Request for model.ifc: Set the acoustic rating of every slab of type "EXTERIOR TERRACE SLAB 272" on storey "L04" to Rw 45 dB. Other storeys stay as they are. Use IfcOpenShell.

First a look at what the model holds.

```python
import ifcopenshell
import ifcopenshell.util.element

model = ifcopenshell.open("model.ifc")
print(model.schema)
storey = next(s for s in model.by_type("IfcBuildingStorey") if s.Name == "L04")
slabs = [e for e in ifcopenshell.util.element.get_decomposition(storey) if e.is_a("IfcSlab")]
seen = {}
for e in slabs:
    element_type = ifcopenshell.util.element.get_type(e)
    key = (element_type.Name if element_type != e and element_type else None, ifcopenshell.util.element.get_pset(e, "Pset_SlabCommon", "AcousticRating"))
    seen[key] = seen.get(key, 0) + 1
for (name, value), count in sorted(seen.items(), key=str):
    print(count, "x", name, "|", value)
```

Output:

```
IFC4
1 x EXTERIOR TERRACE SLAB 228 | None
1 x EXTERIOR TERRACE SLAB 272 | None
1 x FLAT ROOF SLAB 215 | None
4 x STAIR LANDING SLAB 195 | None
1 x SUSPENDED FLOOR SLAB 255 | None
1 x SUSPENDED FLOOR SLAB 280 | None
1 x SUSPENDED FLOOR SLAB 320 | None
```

```python
import ifcopenshell
import ifcopenshell.api.pset
import ifcopenshell.util.element

model = ifcopenshell.open("model.ifc")

storey = next(s for s in model.by_type("IfcBuildingStorey") if s.Name == "L04")
slabs = [e for e in ifcopenshell.util.element.get_decomposition(storey) if e.is_a("IfcSlab")]

count = 0
for e in slabs:
    element_type = ifcopenshell.util.element.get_type(e)
    if element_type in (None, e) or element_type.Name != "EXTERIOR TERRACE SLAB 272":
        continue
    # add_pset returns the element's existing set when there is one.
    pset = ifcopenshell.api.pset.add_pset(model, product=e, name="Pset_SlabCommon")
    ifcopenshell.api.pset.edit_pset(model, pset=pset, properties={"AcousticRating": "Rw 45 dB"})
    count += 1

print(count, "slabs updated")

model.write("model_rev.ifc")
```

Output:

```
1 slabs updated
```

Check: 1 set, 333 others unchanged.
